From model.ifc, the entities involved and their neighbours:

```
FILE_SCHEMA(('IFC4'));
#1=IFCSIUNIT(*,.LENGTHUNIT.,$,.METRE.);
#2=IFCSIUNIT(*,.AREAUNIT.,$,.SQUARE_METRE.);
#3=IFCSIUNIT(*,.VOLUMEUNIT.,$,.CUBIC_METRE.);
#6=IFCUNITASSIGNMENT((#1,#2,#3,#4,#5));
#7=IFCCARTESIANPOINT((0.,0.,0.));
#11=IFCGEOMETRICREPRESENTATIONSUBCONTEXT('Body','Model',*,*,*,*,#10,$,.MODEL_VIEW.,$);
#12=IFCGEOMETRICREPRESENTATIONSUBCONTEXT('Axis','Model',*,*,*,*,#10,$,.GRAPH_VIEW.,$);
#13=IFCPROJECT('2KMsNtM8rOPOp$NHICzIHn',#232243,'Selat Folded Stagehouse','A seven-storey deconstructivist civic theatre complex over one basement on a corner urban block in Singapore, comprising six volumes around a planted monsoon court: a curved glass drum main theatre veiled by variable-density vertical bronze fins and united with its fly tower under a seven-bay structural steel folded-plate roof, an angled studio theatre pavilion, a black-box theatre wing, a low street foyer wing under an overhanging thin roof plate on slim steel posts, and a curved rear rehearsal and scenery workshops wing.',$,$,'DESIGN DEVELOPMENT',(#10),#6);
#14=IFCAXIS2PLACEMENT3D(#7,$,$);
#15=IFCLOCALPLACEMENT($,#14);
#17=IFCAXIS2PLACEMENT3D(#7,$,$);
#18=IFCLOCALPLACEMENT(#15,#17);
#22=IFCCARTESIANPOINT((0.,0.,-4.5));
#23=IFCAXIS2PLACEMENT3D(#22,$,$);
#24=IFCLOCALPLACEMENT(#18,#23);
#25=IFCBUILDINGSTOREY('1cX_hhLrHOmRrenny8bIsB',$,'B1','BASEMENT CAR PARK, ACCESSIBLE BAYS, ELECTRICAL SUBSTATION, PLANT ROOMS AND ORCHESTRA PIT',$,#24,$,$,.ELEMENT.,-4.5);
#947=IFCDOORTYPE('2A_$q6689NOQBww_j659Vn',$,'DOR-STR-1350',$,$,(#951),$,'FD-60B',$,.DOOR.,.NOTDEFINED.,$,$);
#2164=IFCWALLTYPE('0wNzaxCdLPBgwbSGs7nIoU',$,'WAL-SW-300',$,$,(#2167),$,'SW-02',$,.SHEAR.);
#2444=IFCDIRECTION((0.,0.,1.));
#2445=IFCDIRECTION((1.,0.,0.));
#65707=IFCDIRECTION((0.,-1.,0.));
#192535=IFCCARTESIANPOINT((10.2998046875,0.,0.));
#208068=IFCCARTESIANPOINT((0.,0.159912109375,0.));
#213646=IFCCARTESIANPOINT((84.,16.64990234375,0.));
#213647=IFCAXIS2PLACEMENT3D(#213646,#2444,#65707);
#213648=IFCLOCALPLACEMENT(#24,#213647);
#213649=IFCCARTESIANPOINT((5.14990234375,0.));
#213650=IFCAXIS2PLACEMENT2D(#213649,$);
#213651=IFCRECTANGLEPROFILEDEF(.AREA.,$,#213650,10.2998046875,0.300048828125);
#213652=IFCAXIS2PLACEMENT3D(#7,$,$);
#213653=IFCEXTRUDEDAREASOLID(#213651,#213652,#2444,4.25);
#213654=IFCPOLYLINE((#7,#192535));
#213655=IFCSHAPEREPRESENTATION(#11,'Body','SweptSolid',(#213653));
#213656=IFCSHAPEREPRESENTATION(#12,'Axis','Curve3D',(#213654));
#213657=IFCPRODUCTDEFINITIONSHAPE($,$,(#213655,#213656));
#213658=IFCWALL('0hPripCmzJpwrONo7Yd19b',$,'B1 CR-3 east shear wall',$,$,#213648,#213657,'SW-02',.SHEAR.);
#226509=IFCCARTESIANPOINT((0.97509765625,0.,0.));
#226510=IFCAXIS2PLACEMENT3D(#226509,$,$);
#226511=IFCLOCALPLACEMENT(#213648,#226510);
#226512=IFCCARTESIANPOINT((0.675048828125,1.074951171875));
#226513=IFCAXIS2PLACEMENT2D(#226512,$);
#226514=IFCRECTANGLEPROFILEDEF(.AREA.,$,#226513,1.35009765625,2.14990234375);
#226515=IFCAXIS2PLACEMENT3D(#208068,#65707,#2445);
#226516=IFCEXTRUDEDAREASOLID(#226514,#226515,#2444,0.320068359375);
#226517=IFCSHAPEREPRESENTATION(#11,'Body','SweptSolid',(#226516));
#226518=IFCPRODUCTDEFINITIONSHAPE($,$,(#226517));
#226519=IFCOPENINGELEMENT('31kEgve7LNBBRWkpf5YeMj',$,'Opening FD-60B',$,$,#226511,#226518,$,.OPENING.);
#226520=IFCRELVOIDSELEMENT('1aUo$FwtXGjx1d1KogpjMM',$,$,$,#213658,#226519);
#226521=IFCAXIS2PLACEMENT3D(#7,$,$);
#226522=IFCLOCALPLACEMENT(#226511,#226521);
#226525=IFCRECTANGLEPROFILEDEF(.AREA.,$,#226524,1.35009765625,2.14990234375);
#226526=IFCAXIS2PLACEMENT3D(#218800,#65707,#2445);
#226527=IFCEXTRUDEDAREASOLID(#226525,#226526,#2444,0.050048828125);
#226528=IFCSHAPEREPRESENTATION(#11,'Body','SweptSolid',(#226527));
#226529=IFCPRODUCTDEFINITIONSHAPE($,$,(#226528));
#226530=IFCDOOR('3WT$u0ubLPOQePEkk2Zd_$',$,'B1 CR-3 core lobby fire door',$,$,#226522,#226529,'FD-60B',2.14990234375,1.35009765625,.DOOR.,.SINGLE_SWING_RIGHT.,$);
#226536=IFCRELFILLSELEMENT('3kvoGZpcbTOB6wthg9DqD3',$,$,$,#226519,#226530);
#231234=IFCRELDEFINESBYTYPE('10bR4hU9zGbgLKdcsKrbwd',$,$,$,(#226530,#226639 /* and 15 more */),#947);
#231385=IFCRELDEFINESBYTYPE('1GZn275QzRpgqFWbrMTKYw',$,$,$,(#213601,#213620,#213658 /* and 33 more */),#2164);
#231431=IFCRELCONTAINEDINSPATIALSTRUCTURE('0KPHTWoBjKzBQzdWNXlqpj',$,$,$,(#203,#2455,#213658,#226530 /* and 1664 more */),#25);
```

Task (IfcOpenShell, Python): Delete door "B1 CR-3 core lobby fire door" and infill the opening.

```python
import ifcopenshell
import ifcopenshell.api.feature
import ifcopenshell.api.root
import ifcopenshell.geom
import ifcopenshell.util.shape

model = ifcopenshell.open("model.ifc")
settings = ifcopenshell.geom.settings()


def volume(element):
    """Net volume in cubic metres, openings subtracted."""
    shape = ifcopenshell.geom.create_shape(settings, element)
    return ifcopenshell.util.shape.get_volume(shape.geometry)


door = model.by_guid("3WT$u0ubLPOQePEkk2Zd_$")
opening = door.FillsVoids[0].RelatingOpeningElement
wall = opening.VoidsElements[0].RelatingBuildingElement
before = volume(wall)

ifcopenshell.api.root.remove_product(model, product=door)
ifcopenshell.api.feature.remove_feature(model, feature=opening)

after = volume(wall)

print(f"wall volume {before:.3f} -> {after:.3f} m3")

model.write("model_edited.ifc")
```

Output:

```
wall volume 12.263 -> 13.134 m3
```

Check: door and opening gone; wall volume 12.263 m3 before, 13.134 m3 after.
